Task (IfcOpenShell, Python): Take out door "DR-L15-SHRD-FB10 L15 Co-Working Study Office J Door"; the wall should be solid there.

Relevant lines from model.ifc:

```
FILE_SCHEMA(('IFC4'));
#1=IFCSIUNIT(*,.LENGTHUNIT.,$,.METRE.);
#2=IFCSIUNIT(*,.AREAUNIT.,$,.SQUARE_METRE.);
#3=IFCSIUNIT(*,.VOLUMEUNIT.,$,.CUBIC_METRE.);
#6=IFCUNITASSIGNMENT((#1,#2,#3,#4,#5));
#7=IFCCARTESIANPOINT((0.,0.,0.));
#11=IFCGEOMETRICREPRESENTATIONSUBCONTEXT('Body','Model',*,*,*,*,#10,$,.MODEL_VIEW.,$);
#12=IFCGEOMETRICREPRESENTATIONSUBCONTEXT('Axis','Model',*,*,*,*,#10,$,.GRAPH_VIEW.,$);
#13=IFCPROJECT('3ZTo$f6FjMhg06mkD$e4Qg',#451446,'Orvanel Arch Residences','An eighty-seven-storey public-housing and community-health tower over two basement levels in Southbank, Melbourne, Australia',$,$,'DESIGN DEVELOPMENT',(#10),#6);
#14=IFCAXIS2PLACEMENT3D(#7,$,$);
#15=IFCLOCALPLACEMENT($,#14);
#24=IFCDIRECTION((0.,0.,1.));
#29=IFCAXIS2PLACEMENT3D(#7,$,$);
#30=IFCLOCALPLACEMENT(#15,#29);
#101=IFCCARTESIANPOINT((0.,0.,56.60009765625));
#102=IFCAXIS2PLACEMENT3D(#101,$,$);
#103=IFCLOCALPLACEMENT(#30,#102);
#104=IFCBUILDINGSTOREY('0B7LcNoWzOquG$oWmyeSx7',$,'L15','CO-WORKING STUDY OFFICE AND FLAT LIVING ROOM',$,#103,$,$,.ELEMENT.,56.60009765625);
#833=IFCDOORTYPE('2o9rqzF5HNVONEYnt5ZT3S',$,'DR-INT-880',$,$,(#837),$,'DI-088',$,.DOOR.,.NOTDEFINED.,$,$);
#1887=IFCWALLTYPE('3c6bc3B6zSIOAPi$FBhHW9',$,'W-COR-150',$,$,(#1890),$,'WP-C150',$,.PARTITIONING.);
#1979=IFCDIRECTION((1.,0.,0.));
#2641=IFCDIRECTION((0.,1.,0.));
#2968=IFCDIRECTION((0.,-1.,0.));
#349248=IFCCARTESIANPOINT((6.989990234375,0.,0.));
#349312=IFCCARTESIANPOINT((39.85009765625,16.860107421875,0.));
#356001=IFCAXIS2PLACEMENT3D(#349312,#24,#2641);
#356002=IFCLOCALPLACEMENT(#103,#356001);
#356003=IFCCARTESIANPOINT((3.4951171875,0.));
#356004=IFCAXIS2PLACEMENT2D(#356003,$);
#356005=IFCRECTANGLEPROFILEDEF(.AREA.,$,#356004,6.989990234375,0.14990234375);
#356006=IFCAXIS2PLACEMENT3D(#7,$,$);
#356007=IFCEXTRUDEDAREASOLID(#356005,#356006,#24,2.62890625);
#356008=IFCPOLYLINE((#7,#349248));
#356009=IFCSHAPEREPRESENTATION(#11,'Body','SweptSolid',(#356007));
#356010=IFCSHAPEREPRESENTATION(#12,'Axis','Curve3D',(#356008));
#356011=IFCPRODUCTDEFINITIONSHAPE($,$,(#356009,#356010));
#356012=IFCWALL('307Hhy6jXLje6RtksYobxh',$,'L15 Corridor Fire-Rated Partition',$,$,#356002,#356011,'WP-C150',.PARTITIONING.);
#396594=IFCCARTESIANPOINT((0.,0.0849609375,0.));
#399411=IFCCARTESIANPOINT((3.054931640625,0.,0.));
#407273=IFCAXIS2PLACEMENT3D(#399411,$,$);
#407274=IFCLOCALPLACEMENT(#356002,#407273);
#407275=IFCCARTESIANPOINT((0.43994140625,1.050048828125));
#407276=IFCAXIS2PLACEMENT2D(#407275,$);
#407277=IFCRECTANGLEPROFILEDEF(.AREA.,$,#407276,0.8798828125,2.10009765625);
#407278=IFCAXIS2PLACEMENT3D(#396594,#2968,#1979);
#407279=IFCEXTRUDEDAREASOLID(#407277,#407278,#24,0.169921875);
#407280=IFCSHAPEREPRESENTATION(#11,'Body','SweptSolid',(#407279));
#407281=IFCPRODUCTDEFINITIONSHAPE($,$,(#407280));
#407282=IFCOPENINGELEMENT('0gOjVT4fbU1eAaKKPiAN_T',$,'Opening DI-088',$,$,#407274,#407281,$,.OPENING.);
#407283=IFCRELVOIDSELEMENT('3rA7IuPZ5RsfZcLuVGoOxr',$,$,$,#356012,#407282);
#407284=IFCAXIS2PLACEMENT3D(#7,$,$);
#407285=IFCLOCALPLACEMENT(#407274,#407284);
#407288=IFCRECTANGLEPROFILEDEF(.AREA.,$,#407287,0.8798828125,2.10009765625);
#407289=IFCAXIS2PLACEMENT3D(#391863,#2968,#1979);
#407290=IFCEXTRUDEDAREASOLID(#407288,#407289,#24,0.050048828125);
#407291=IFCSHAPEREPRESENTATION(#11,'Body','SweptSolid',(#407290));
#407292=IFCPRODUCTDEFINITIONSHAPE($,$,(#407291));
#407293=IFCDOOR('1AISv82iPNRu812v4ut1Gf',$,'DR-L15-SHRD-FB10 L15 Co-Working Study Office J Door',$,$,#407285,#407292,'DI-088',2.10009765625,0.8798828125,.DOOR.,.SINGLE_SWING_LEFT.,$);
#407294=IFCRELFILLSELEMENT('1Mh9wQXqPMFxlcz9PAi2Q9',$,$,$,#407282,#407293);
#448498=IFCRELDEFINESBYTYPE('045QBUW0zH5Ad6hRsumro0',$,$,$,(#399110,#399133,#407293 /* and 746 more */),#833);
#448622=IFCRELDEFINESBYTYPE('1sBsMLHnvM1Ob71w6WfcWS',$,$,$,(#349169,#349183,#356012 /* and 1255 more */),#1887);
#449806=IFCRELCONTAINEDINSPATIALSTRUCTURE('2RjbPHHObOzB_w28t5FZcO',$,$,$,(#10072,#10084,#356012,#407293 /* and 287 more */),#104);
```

```python
import ifcopenshell
import ifcopenshell.api.feature
import ifcopenshell.api.root
import ifcopenshell.geom
import ifcopenshell.util.shape

model = ifcopenshell.open("model.ifc")
settings = ifcopenshell.geom.settings()


def volume(element):
    """Net volume in cubic metres, openings subtracted."""
    shape = ifcopenshell.geom.create_shape(settings, element)
    return ifcopenshell.util.shape.get_volume(shape.geometry)


door = model.by_id(407293)
opening = door.FillsVoids[0].RelatingOpeningElement
wall = opening.VoidsElements[0].RelatingBuildingElement
before = volume(wall)

ifcopenshell.api.root.remove_product(model, product=door)
ifcopenshell.api.feature.remove_feature(model, feature=opening)

after = volume(wall)

print(f"wall volume {before:.3f} -> {after:.3f} m3")

model.write("model_rev.ifc")
```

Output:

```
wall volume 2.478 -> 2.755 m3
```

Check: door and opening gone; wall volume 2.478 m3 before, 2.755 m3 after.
